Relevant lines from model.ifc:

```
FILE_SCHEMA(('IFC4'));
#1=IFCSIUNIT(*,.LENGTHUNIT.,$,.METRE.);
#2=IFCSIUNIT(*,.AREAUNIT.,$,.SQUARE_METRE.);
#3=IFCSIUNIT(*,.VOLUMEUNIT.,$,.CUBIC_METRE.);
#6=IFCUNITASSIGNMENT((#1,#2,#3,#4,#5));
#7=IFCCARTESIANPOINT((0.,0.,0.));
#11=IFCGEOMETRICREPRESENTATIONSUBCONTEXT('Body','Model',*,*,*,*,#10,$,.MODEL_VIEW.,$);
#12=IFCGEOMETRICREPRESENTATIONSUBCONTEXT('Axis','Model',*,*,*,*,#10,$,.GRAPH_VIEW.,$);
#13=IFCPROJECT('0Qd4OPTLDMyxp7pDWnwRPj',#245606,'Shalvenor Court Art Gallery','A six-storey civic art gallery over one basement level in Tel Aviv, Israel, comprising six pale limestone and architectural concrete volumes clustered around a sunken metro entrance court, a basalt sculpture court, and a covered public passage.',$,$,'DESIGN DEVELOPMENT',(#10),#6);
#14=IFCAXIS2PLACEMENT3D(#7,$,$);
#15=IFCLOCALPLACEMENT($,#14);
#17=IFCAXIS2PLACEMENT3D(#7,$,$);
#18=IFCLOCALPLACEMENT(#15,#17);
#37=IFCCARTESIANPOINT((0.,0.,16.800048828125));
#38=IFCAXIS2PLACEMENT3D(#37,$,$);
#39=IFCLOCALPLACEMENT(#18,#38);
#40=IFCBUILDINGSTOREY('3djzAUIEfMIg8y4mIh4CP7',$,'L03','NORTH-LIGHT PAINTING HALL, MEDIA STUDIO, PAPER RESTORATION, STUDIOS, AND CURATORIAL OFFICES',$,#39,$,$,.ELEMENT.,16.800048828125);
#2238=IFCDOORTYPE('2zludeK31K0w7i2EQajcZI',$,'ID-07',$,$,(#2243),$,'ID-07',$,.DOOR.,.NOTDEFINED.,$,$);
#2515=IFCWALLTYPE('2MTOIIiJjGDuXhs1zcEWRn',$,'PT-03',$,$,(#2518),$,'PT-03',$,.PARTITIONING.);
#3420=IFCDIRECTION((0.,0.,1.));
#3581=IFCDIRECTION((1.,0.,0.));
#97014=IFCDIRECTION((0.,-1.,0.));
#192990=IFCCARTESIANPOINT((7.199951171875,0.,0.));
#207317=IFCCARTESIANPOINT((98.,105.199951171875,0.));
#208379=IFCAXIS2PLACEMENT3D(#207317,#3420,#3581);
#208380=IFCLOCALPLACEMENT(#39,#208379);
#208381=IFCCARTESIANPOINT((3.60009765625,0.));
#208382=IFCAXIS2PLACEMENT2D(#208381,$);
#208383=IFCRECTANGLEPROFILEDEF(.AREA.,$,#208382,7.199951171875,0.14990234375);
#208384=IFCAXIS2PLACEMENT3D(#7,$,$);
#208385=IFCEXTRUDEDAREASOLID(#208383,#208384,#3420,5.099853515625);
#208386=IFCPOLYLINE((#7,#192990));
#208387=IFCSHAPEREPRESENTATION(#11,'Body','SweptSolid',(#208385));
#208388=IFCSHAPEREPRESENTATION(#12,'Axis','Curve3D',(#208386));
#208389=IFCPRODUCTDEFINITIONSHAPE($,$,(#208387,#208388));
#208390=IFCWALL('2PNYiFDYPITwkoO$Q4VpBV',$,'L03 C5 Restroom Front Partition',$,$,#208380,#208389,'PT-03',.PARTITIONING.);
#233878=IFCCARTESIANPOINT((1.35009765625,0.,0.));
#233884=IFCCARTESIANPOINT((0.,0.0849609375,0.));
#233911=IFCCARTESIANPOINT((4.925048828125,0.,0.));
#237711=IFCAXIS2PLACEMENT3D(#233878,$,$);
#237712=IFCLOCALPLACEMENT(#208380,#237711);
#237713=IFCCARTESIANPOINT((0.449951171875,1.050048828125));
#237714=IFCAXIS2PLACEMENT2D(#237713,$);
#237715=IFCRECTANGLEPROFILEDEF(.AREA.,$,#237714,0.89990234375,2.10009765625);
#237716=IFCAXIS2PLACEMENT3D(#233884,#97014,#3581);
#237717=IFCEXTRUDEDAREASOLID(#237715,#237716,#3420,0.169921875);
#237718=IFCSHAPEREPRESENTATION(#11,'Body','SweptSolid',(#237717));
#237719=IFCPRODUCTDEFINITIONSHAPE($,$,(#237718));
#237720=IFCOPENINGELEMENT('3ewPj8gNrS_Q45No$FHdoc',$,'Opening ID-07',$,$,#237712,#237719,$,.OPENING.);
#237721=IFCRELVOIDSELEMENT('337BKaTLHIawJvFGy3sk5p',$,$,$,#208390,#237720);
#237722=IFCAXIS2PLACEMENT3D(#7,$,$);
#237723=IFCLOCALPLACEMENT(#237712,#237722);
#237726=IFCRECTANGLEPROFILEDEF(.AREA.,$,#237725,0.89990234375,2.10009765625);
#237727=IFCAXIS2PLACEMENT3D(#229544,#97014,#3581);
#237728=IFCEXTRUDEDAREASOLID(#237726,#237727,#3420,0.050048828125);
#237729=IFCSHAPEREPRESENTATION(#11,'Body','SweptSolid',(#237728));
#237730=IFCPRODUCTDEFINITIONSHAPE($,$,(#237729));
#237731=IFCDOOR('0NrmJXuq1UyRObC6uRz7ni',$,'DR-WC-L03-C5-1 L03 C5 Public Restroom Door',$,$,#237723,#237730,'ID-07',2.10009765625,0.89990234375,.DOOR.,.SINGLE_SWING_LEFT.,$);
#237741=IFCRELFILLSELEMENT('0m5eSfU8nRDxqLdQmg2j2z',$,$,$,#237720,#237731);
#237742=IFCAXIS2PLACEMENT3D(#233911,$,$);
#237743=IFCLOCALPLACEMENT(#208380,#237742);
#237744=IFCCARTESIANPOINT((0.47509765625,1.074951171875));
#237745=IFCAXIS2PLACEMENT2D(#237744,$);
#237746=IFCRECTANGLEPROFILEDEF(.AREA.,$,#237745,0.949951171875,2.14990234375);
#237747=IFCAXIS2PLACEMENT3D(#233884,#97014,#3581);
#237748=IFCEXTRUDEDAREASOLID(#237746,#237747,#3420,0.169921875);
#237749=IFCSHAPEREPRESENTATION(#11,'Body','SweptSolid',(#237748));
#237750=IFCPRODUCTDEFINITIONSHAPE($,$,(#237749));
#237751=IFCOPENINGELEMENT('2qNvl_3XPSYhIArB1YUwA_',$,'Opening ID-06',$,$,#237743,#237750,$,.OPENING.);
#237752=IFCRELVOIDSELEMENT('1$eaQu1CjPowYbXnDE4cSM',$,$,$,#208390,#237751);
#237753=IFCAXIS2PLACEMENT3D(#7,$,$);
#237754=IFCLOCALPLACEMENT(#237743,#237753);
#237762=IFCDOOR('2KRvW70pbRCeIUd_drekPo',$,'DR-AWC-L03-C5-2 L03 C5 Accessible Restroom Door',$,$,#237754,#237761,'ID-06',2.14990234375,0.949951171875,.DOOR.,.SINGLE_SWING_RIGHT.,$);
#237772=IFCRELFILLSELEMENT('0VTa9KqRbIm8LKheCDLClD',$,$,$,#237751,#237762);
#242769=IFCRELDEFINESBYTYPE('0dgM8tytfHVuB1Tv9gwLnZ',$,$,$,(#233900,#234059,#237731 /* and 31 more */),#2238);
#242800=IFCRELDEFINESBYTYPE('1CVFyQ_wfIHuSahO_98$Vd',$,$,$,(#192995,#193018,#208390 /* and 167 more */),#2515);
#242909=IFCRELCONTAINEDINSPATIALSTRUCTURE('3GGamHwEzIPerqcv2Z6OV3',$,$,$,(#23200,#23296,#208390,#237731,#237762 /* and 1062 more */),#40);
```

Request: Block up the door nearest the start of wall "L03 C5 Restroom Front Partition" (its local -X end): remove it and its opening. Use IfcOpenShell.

```python
import ifcopenshell
import ifcopenshell.api.feature
import ifcopenshell.api.root
import ifcopenshell.geom
import ifcopenshell.util.shape

model = ifcopenshell.open("model.ifc")
settings = ifcopenshell.geom.settings()


def volume(element):
    """Net volume in cubic metres, openings subtracted."""
    shape = ifcopenshell.geom.create_shape(settings, element)
    return ifcopenshell.util.shape.get_volume(shape.geometry)


door = model.by_guid("0NrmJXuq1UyRObC6uRz7ni")
opening = door.FillsVoids[0].RelatingOpeningElement
wall = opening.VoidsElements[0].RelatingBuildingElement
before = volume(wall)

ifcopenshell.api.root.remove_product(model, product=door)
ifcopenshell.api.feature.remove_feature(model, feature=opening)

after = volume(wall)

print(f"wall volume {before:.3f} -> {after:.3f} m3")

model.write("model_v2.ifc")
```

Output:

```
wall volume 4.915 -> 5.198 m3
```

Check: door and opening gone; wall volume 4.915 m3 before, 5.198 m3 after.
